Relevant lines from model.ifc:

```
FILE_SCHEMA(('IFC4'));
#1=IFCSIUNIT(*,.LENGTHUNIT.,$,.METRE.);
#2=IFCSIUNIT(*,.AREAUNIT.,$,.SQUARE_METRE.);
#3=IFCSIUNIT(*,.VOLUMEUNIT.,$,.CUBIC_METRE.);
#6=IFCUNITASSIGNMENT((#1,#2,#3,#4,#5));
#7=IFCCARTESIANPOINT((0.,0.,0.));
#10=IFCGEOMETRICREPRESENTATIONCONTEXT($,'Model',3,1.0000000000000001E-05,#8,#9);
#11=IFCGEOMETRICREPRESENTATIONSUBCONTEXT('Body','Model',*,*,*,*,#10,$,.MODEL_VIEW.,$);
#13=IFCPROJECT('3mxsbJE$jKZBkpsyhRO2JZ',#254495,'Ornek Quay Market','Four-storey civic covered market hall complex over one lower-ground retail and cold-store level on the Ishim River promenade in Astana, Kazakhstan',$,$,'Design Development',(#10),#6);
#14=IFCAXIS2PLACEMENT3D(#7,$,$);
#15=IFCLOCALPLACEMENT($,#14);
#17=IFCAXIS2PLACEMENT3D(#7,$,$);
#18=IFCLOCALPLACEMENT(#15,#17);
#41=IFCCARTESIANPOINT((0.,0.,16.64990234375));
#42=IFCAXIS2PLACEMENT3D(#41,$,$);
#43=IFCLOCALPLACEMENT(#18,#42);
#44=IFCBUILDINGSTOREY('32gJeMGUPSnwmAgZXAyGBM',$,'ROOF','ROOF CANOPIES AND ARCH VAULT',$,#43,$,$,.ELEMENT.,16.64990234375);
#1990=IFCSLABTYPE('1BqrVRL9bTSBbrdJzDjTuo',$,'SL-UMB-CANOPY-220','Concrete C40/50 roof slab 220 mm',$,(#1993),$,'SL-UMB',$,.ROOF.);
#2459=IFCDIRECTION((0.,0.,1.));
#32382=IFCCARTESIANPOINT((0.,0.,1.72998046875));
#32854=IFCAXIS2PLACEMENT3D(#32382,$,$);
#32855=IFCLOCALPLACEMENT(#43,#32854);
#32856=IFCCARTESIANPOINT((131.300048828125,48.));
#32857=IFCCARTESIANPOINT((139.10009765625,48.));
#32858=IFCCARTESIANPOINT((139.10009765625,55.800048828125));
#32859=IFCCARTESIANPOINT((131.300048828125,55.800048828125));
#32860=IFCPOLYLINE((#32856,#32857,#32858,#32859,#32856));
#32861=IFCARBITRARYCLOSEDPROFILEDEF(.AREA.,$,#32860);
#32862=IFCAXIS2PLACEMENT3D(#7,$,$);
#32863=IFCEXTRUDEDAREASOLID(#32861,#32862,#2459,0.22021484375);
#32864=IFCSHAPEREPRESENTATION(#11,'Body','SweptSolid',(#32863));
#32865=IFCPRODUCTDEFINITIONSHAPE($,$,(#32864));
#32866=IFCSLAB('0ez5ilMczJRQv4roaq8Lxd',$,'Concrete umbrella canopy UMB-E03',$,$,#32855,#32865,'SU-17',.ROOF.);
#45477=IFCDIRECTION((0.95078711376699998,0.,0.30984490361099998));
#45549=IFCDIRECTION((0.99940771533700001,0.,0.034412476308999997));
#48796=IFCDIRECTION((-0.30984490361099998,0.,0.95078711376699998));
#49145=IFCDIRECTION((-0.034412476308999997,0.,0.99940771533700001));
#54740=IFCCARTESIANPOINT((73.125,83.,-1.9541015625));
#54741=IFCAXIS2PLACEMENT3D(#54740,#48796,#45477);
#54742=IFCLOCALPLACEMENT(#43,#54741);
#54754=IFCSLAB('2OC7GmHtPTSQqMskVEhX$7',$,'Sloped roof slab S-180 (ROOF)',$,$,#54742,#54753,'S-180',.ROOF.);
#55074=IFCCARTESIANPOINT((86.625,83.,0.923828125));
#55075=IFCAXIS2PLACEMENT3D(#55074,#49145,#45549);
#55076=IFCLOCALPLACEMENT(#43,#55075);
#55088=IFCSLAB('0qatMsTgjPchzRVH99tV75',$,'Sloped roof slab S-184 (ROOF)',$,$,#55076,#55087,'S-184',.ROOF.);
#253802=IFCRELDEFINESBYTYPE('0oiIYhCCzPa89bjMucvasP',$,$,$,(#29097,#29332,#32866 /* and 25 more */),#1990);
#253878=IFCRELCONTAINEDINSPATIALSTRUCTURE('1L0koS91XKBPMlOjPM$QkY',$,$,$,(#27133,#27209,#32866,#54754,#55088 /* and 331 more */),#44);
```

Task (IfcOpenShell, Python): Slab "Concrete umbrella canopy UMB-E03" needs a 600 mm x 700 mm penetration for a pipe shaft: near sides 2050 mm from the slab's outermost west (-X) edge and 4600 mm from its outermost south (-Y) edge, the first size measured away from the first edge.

```python
import numpy as np
import ifcopenshell
import ifcopenshell.api.feature
import ifcopenshell.api.geometry
import ifcopenshell.api.root
import ifcopenshell.geom
import ifcopenshell.util.placement
import ifcopenshell.util.representation
import ifcopenshell.util.shape
import ifcopenshell.util.unit

model = ifcopenshell.open("model.ifc")
unit_scale = ifcopenshell.util.unit.calculate_unit_scale(model)
settings = ifcopenshell.geom.settings()


def volume(element):
    """Net volume in cubic metres, openings subtracted."""
    shape = ifcopenshell.geom.create_shape(settings, element)
    return ifcopenshell.util.shape.get_volume(shape.geometry)


slab = model.by_guid("0ez5ilMczJRQv4roaq8Lxd")
before = volume(slab)

# Extent in the slab's own axes, in metres. The edges named are its -X and -Y sides.
slab_shape = ifcopenshell.geom.create_shape(settings, slab)
vertices = ifcopenshell.util.shape.get_vertices(slab_shape.geometry)
x_min, y_min, bottom = vertices.min(axis=0)
top = vertices[:, 2].max()

opening = ifcopenshell.api.root.create_entity(model, ifc_class="IfcOpeningElement", name="Pipe shaft opening", predefined_type="OPENING")
context = ifcopenshell.util.representation.get_context(model, "Model", "Body", "MODEL_VIEW")
width, depth = 0.6, 0.7
outline = [(0.0, 0.0), (width, 0.0), (width, depth), (0.0, depth), (0.0, 0.0)]
# Overshoot both faces by 50 mm so the cut is clean.
shape = ifcopenshell.api.geometry.add_slab_representation(
    model, context=context, depth=top - bottom + 0.1, polyline=outline
)
ifcopenshell.api.geometry.assign_representation(model, product=opening, representation=shape)

matrix = ifcopenshell.util.placement.get_local_placement(slab.ObjectPlacement)
matrix[:, 3] = matrix @ np.append(np.array([x_min + 2.05, y_min + 4.6, bottom - 0.05]) / unit_scale, 1.0)
ifcopenshell.api.geometry.edit_object_placement(model, product=opening, matrix=matrix, is_si=False)
ifcopenshell.api.feature.add_feature(model, feature=opening, element=slab)

after = volume(slab)

print(f"slab volume {before:.3f} -> {after:.3f} m3")

model.write("model-out.ifc")
```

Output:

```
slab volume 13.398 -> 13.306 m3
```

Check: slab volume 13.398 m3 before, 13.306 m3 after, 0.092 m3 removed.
